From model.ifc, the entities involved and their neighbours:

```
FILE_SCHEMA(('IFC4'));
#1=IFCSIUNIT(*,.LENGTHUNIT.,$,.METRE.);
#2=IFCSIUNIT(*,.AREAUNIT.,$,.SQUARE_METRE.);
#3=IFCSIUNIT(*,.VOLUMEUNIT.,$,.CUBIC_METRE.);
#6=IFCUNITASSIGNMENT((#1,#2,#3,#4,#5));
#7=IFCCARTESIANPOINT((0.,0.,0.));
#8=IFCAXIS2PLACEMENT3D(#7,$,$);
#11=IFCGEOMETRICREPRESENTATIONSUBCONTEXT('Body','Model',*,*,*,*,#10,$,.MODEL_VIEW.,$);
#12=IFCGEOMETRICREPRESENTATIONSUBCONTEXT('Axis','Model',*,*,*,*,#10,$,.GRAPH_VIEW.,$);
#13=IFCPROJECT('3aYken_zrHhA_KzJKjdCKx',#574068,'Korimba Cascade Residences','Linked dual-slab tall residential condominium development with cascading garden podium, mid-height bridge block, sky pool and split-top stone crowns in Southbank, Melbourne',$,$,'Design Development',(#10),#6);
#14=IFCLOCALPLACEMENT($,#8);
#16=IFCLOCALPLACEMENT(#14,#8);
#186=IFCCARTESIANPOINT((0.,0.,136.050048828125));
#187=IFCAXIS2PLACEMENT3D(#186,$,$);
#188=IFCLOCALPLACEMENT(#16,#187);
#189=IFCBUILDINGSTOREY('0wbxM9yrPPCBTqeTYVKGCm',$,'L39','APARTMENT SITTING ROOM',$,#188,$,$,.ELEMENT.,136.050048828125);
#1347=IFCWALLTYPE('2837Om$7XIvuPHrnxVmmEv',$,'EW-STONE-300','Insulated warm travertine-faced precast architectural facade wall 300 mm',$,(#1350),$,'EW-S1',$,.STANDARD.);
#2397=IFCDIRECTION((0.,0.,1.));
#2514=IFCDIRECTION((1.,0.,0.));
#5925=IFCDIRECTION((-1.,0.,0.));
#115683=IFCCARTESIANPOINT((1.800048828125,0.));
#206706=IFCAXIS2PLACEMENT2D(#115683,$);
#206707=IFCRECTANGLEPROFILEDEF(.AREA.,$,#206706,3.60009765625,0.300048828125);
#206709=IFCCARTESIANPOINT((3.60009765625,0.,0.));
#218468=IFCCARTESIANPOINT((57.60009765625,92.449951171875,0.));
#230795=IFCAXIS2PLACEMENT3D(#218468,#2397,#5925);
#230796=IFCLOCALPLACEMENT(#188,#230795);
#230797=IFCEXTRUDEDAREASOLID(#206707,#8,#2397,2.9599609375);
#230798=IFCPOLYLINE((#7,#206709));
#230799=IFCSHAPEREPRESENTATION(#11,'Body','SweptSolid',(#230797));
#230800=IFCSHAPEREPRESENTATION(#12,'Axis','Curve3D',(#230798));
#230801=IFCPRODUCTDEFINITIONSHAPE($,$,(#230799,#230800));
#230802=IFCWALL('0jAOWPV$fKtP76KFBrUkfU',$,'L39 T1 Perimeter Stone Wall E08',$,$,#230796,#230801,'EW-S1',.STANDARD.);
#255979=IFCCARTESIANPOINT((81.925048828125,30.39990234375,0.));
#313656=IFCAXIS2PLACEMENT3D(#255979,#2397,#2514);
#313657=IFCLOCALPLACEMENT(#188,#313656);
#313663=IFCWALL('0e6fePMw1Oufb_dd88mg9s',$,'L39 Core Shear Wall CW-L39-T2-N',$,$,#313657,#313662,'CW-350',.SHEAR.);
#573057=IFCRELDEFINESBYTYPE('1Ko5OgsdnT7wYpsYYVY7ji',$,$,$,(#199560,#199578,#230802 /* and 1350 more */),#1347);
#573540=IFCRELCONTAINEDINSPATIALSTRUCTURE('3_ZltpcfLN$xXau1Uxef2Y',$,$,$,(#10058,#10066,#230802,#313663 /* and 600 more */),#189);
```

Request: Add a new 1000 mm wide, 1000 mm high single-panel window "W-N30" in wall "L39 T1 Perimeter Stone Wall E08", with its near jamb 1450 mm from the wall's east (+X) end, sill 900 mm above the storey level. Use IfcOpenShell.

```python
import numpy as np
import ifcopenshell
import ifcopenshell.api.feature
import ifcopenshell.api.geometry
import ifcopenshell.api.root
import ifcopenshell.api.spatial
import ifcopenshell.geom
import ifcopenshell.util.element
import ifcopenshell.util.placement
import ifcopenshell.util.representation
import ifcopenshell.util.shape
import ifcopenshell.util.unit

model = ifcopenshell.open("model.ifc")
unit_scale = ifcopenshell.util.unit.calculate_unit_scale(model)
settings = ifcopenshell.geom.settings()


def volume(element):
    """Net volume in cubic metres, openings subtracted."""
    shape = ifcopenshell.geom.create_shape(settings, element)
    return ifcopenshell.util.shape.get_volume(shape.geometry)


wall = model.by_guid("0jAOWPV$fKtP76KFBrUkfU")
storey = ifcopenshell.util.element.get_container(wall, ifc_class="IfcBuildingStorey")
context = ifcopenshell.util.representation.get_context(model, "Model", "Body", "MODEL_VIEW")
before = volume(wall)

width, height, from_end, sill = 1, 1, 1.45, 0.9  # metres

# The wall runs along its own X axis, and the end named is its -X end.
wall_shape = ifcopenshell.geom.create_shape(settings, wall)
x, y, z = ifcopenshell.util.shape.get_vertices(wall_shape.geometry).T
start = x.min() + from_end
face, thickness = float(y.min()), float(y.max() - y.min())
wall_matrix = ifcopenshell.util.placement.get_local_placement(wall.ObjectPlacement)
level = ifcopenshell.util.placement.get_local_placement(storey.ObjectPlacement)[2, 3]


def in_wall(x, y):
    """Placement at x, y metres in the wall's axes, at sill height."""
    matrix = wall_matrix.copy()
    matrix[:, 3] = wall_matrix @ np.array([x / unit_scale, y / unit_scale, 0.0, 1.0])
    matrix[2, 3] = level + sill / unit_scale
    return matrix


# Opening: a box that overshoots both wall faces by 50 mm.
opening = ifcopenshell.api.root.create_entity(model, ifc_class="IfcOpeningElement", predefined_type="OPENING")
box = ifcopenshell.api.geometry.add_wall_representation(
    model, context=context, length=width, height=height, thickness=thickness + 0.1
)
ifcopenshell.api.geometry.assign_representation(model, product=opening, representation=box)
ifcopenshell.api.geometry.edit_object_placement(model, product=opening, matrix=in_wall(start, face - 0.05), is_si=False)
ifcopenshell.api.feature.add_feature(model, feature=opening, element=wall)

window = ifcopenshell.api.root.create_entity(model, ifc_class="IfcWindow", name="W-N30", predefined_type="WINDOW")
window.OverallWidth, window.OverallHeight = width / unit_scale, height / unit_scale
window.PartitioningType = "SINGLE_PANEL"
body = ifcopenshell.api.geometry.add_window_representation(
    model,
    context=context,
    overall_width=window.OverallWidth,
    overall_height=window.OverallHeight,
    partition_type="SINGLE_PANEL",
)
ifcopenshell.api.geometry.assign_representation(model, product=window, representation=body)
ifcopenshell.api.spatial.assign_container(model, products=[window], relating_structure=storey)
ifcopenshell.api.feature.add_filling(model, opening=opening, element=window)

# Centre the window in the wall's thickness.
ifcopenshell.api.geometry.edit_object_placement(model, product=window, matrix=in_wall(start, face), is_si=False)
window_shape = ifcopenshell.geom.create_shape(settings, window)
depth = ifcopenshell.util.shape.get_vertices(window_shape.geometry)[:, 1]
offset = face + thickness / 2 - (depth.min() + depth.max()) / 2
ifcopenshell.api.geometry.edit_object_placement(model, product=window, matrix=in_wall(start, offset), is_si=False)

after = volume(wall)

print(f"wall volume {before:.3f} -> {after:.3f} m3")

model.write("model_edited.ifc")
```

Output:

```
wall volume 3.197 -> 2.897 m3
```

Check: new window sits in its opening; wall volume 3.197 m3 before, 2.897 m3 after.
